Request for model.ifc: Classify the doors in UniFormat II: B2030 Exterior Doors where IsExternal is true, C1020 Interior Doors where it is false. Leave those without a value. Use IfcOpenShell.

First a look at what the model holds.

```python
import ifcopenshell
import ifcopenshell.util.element

model = ifcopenshell.open("model.ifc")
print(model.schema)
print("classifications:", [c.Name for c in model.by_type("IfcClassification")])
values = [ifcopenshell.util.element.get_pset(e, "Pset_DoorCommon", "IsExternal") for e in model.by_type("IfcDoor")]
for value in (True, False, None):
    print("IsExternal", value, values.count(value))
```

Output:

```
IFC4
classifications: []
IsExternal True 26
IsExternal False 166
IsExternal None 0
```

```python
import ifcopenshell
import ifcopenshell.api.classification
import ifcopenshell.util.element

model = ifcopenshell.open("model.ifc")

system = ifcopenshell.api.classification.add_classification(model, classification="UniFormat II")

doors = model.by_type("IfcDoor")
external = {e: ifcopenshell.util.element.get_pset(e, "Pset_DoorCommon", "IsExternal") for e in doors}
for flag, code, name in ((True, "B2030", "Exterior Doors"), (False, "C1020", "Interior Doors")):
    products = [e for e in doors if external[e] is flag]
    ifcopenshell.api.classification.add_reference(
        model, products=products, classification=system, identification=code, name=name
    )
    print(code, len(products))

model.write("model_edited.ifc")
```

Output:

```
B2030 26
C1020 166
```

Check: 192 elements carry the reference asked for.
